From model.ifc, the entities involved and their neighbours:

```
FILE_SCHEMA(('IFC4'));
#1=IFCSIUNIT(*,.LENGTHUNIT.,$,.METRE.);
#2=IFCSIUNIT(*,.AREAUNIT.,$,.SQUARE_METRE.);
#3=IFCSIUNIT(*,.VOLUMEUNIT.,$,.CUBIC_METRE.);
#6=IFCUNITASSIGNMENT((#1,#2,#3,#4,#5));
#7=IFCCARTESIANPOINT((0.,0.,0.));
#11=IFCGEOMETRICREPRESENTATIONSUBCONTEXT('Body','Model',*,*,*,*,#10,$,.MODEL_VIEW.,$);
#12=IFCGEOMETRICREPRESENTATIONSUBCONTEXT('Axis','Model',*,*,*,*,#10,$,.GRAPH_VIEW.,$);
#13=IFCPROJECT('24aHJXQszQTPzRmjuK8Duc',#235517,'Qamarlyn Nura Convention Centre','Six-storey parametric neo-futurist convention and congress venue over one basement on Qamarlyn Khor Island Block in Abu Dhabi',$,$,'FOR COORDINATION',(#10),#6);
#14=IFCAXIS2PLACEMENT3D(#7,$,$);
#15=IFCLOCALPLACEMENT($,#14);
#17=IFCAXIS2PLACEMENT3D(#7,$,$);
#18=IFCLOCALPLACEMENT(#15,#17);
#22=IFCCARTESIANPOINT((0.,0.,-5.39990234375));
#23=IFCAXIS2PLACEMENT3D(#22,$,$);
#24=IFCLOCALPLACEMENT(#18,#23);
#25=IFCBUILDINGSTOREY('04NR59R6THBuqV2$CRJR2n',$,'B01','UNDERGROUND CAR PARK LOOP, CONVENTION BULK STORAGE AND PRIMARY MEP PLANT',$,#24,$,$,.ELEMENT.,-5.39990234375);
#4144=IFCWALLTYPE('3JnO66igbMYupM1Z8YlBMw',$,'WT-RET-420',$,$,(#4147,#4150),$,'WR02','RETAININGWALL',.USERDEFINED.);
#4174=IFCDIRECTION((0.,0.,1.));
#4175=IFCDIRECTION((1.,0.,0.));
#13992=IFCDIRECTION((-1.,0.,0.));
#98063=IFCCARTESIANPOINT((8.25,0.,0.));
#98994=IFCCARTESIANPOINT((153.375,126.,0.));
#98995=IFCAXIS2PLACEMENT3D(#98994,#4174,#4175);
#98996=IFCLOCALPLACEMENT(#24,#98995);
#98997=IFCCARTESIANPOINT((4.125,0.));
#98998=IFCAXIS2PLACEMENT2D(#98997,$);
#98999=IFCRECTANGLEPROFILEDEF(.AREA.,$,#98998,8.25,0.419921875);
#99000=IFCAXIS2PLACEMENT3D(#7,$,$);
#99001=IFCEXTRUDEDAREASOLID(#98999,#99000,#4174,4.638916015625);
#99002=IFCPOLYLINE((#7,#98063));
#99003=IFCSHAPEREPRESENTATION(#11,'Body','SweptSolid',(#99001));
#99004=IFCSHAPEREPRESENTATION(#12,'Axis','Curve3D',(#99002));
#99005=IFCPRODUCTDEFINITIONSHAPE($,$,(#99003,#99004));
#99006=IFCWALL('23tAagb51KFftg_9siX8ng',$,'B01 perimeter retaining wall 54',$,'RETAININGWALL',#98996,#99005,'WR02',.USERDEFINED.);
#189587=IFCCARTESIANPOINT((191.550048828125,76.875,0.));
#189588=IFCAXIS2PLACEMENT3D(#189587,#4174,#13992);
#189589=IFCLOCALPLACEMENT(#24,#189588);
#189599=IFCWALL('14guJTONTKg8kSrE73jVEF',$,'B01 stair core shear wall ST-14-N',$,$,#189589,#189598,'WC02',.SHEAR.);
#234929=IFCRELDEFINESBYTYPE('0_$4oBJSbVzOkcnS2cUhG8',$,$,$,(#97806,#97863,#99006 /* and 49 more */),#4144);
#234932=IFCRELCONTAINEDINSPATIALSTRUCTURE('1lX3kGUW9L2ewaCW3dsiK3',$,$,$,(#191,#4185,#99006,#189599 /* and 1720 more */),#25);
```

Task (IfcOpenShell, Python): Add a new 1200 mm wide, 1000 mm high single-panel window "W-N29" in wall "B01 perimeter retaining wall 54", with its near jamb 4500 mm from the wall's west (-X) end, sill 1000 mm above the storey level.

```python
import numpy as np
import ifcopenshell
import ifcopenshell.api.feature
import ifcopenshell.api.geometry
import ifcopenshell.api.root
import ifcopenshell.api.spatial
import ifcopenshell.geom
import ifcopenshell.util.element
import ifcopenshell.util.placement
import ifcopenshell.util.representation
import ifcopenshell.util.shape
import ifcopenshell.util.unit

model = ifcopenshell.open("model.ifc")
unit_scale = ifcopenshell.util.unit.calculate_unit_scale(model)
settings = ifcopenshell.geom.settings()


def volume(element):
    """Net volume in cubic metres, openings subtracted."""
    shape = ifcopenshell.geom.create_shape(settings, element)
    return ifcopenshell.util.shape.get_volume(shape.geometry)


wall = model.by_guid("23tAagb51KFftg_9siX8ng")
storey = ifcopenshell.util.element.get_container(wall, ifc_class="IfcBuildingStorey")
context = ifcopenshell.util.representation.get_context(model, "Model", "Body", "MODEL_VIEW")
before = volume(wall)

width, height, from_end, sill = 1.2, 1, 4.5, 1  # metres

# The wall runs along its own X axis, and the end named is its -X end.
wall_shape = ifcopenshell.geom.create_shape(settings, wall)
x, y, z = ifcopenshell.util.shape.get_vertices(wall_shape.geometry).T
start = x.min() + from_end
face, thickness = float(y.min()), float(y.max() - y.min())
wall_matrix = ifcopenshell.util.placement.get_local_placement(wall.ObjectPlacement)
level = ifcopenshell.util.placement.get_local_placement(storey.ObjectPlacement)[2, 3]


def in_wall(x, y):
    """Placement at x, y metres in the wall's axes, at sill height."""
    matrix = wall_matrix.copy()
    matrix[:, 3] = wall_matrix @ np.array([x / unit_scale, y / unit_scale, 0.0, 1.0])
    matrix[2, 3] = level + sill / unit_scale
    return matrix


# Opening: a box that overshoots both wall faces by 50 mm.
opening = ifcopenshell.api.root.create_entity(model, ifc_class="IfcOpeningElement", predefined_type="OPENING")
box = ifcopenshell.api.geometry.add_wall_representation(
    model, context=context, length=width, height=height, thickness=thickness + 0.1
)
ifcopenshell.api.geometry.assign_representation(model, product=opening, representation=box)
ifcopenshell.api.geometry.edit_object_placement(model, product=opening, matrix=in_wall(start, face - 0.05), is_si=False)
ifcopenshell.api.feature.add_feature(model, feature=opening, element=wall)

window = ifcopenshell.api.root.create_entity(model, ifc_class="IfcWindow", name="W-N29", predefined_type="WINDOW")
window.OverallWidth, window.OverallHeight = width / unit_scale, height / unit_scale
window.PartitioningType = "SINGLE_PANEL"
body = ifcopenshell.api.geometry.add_window_representation(
    model,
    context=context,
    overall_width=window.OverallWidth,
    overall_height=window.OverallHeight,
    partition_type="SINGLE_PANEL",
)
ifcopenshell.api.geometry.assign_representation(model, product=window, representation=body)
ifcopenshell.api.spatial.assign_container(model, products=[window], relating_structure=storey)
ifcopenshell.api.feature.add_filling(model, opening=opening, element=window)

# Centre the window in the wall's thickness.
ifcopenshell.api.geometry.edit_object_placement(model, product=window, matrix=in_wall(start, face), is_si=False)
window_shape = ifcopenshell.geom.create_shape(settings, window)
depth = ifcopenshell.util.shape.get_vertices(window_shape.geometry)[:, 1]
offset = face + thickness / 2 - (depth.min() + depth.max()) / 2
ifcopenshell.api.geometry.edit_object_placement(model, product=window, matrix=in_wall(start, offset), is_si=False)

after = volume(wall)

print(f"wall volume {before:.3f} -> {after:.3f} m3")

model.write("model_updated.ifc")
```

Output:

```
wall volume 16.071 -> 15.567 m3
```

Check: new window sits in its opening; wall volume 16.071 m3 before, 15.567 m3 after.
